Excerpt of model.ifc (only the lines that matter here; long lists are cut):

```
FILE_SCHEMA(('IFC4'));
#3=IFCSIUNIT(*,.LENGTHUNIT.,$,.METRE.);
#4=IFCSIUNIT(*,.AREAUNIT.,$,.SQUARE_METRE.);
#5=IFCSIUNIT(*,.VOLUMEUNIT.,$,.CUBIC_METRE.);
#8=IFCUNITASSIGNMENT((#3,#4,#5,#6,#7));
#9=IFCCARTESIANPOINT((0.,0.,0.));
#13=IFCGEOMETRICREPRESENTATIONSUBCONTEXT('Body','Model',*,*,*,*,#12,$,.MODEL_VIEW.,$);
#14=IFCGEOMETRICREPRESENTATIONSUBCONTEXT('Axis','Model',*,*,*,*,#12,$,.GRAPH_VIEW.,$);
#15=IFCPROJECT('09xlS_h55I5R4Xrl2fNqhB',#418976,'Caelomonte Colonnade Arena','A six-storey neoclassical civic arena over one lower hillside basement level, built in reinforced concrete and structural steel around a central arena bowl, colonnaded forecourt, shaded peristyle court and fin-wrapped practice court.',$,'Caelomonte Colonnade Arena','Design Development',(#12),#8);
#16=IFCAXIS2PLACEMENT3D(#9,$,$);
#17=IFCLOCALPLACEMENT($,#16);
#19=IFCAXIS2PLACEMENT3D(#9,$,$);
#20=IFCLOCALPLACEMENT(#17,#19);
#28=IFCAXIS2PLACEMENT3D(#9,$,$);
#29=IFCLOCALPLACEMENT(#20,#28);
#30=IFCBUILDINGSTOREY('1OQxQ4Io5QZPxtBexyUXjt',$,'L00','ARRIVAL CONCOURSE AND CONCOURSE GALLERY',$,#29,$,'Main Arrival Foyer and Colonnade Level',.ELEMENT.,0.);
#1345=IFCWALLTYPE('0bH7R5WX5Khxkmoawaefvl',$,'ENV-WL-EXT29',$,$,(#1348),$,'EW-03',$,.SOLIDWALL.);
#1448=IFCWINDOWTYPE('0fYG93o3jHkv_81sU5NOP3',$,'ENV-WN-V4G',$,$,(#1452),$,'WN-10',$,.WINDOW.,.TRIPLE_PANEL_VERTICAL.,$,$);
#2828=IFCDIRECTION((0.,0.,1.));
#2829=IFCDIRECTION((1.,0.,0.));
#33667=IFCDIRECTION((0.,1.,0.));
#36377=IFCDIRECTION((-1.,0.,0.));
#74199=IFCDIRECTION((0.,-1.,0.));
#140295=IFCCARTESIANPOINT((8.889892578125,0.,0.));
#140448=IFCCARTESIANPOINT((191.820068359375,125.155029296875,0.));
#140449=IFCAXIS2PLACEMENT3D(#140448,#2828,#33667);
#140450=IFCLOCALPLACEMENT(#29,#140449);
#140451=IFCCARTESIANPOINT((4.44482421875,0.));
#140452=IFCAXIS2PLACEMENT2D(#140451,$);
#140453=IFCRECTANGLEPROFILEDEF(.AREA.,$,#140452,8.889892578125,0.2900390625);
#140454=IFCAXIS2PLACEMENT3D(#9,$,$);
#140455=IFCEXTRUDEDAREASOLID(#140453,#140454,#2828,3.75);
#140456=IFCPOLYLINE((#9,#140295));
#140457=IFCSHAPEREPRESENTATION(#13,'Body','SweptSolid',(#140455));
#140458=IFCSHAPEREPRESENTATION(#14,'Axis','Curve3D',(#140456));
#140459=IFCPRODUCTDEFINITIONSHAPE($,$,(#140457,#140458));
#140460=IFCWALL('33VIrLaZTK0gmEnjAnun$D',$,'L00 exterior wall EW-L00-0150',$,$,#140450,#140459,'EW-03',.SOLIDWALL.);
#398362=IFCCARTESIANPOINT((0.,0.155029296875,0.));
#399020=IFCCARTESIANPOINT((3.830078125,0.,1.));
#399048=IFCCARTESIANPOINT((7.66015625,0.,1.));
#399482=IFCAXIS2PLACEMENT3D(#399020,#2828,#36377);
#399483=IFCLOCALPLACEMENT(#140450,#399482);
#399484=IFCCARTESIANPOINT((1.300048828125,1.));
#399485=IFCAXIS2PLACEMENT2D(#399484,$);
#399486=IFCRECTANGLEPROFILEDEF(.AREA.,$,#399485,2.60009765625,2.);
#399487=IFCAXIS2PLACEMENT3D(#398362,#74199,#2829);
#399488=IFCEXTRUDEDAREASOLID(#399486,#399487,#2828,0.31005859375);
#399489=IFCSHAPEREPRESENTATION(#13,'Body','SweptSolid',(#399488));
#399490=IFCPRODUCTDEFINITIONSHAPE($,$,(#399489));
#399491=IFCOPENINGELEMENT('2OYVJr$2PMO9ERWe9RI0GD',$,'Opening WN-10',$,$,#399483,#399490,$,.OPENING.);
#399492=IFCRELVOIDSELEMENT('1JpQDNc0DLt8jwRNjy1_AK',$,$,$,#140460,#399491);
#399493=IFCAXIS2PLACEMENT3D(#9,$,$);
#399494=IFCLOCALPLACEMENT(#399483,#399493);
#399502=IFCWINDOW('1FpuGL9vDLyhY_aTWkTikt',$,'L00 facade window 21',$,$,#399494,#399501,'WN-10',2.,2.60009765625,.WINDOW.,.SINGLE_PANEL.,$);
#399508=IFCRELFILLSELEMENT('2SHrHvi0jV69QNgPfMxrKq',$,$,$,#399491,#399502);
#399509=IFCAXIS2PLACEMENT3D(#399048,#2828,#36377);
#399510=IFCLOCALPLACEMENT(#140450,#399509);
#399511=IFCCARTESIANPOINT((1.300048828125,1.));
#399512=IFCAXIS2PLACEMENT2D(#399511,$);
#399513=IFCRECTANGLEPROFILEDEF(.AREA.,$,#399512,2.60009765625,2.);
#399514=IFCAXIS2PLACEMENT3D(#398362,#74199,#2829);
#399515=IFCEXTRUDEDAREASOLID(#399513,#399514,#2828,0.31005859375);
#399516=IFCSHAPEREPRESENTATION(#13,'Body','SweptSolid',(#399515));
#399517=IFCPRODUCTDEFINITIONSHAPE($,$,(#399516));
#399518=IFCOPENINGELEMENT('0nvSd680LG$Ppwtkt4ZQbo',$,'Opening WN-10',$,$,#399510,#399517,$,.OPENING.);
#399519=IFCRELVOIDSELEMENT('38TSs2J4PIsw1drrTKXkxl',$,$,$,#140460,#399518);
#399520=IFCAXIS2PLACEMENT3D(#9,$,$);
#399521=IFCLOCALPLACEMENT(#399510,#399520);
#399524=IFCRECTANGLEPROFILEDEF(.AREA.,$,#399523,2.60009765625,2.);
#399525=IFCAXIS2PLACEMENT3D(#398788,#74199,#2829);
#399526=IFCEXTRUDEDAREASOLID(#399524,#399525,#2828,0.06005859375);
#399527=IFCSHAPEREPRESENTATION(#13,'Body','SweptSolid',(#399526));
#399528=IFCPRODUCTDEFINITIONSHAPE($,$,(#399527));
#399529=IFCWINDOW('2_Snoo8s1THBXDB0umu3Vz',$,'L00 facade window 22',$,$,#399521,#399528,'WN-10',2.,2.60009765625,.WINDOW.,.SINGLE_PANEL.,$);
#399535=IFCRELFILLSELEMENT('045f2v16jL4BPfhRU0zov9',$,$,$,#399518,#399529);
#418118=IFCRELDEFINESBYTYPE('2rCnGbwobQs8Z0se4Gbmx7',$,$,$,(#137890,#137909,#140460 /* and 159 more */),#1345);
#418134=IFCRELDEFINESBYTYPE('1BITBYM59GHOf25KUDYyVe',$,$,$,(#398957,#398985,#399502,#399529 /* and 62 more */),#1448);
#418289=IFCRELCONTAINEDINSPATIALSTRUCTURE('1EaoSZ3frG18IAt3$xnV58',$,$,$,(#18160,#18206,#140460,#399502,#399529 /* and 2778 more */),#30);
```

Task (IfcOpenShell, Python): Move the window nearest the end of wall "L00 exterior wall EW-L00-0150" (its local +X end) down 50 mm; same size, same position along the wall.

```python
import numpy as np
import ifcopenshell
import ifcopenshell.api.geometry
import ifcopenshell.util.placement
import ifcopenshell.util.unit

model = ifcopenshell.open("model.ifc")
unit_scale = ifcopenshell.util.unit.calculate_unit_scale(model)

window = model.by_guid("2_Snoo8s1THBXDB0umu3Vz")
opening = window.FillsVoids[0].RelatingOpeningElement
dz = -0.05

shift = np.array([0.0, 0.0, dz])
# The window is placed relative to its opening, so it follows when the opening moves.
matrix = ifcopenshell.util.placement.get_local_placement(opening.ObjectPlacement)
matrix[:3, 3] += shift
ifcopenshell.api.geometry.edit_object_placement(
    model, product=opening, matrix=matrix, is_si=False, should_transform_children=True
)

print(f"moved by {dz * unit_scale:+.3f} m")

model.write("model_rev.ifc")
```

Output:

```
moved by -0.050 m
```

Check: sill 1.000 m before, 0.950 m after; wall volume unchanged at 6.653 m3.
